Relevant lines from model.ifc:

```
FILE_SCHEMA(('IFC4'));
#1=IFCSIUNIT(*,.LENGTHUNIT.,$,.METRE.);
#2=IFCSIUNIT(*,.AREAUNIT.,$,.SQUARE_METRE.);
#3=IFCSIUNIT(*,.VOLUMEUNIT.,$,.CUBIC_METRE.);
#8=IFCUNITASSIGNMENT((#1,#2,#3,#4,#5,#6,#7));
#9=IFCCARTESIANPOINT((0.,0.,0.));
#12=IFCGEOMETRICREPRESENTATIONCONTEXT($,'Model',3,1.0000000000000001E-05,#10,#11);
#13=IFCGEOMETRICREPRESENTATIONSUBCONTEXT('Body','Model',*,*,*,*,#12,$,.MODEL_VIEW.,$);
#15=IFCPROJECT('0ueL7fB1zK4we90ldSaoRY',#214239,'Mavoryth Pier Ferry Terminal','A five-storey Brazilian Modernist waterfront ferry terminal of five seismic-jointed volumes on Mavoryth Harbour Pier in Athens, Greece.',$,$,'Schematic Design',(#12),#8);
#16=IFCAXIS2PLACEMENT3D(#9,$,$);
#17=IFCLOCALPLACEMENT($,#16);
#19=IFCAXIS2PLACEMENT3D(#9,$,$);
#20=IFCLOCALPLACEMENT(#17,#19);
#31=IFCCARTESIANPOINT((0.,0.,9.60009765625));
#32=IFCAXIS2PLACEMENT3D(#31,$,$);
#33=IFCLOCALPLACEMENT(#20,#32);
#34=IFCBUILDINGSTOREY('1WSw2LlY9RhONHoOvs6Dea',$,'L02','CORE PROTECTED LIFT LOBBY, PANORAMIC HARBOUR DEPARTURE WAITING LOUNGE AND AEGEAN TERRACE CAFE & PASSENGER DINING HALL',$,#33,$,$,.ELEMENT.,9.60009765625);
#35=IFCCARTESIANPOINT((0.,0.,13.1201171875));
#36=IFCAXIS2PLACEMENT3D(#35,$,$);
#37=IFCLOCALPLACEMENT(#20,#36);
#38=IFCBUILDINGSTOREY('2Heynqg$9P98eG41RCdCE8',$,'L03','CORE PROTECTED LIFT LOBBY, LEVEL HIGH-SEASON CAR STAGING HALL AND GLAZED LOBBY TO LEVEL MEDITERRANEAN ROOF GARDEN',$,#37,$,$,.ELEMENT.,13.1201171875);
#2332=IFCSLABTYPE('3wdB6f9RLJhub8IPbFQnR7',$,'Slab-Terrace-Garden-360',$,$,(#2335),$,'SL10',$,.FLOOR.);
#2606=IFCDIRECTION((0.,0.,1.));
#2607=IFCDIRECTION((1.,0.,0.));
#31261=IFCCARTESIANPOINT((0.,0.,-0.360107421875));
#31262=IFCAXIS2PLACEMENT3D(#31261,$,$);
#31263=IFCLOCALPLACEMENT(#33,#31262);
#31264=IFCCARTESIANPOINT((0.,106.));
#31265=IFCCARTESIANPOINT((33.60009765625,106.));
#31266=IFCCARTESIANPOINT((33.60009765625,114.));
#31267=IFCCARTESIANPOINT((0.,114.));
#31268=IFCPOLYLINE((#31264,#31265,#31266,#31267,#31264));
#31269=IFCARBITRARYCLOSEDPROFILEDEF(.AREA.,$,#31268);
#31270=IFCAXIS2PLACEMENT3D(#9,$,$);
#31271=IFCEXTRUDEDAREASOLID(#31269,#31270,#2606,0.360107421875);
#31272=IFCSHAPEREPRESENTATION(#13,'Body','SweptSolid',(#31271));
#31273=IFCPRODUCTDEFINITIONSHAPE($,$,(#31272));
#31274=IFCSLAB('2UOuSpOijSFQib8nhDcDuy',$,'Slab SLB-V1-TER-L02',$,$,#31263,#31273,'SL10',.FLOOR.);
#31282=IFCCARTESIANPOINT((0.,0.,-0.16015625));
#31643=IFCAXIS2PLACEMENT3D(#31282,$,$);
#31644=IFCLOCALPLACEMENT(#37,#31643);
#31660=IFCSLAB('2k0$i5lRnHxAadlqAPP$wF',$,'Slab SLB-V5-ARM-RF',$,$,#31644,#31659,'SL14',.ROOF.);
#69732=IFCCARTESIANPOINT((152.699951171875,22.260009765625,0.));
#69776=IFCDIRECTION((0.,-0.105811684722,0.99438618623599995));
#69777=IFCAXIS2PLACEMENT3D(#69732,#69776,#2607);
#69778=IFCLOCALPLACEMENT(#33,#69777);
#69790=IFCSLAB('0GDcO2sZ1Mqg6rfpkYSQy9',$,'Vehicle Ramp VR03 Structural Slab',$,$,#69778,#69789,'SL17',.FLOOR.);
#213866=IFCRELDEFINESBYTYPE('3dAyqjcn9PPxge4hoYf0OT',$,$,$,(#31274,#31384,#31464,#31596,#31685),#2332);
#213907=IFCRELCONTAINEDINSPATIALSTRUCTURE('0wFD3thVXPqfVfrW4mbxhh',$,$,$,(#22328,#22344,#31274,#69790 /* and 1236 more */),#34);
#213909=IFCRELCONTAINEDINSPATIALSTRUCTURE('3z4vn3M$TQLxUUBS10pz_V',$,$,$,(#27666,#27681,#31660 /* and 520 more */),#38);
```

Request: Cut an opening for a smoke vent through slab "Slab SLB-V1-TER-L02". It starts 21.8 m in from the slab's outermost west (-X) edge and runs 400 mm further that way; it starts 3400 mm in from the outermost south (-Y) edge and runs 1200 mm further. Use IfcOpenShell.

```python
import numpy as np
import ifcopenshell
import ifcopenshell.api.feature
import ifcopenshell.api.geometry
import ifcopenshell.api.root
import ifcopenshell.geom
import ifcopenshell.util.placement
import ifcopenshell.util.representation
import ifcopenshell.util.shape
import ifcopenshell.util.unit

model = ifcopenshell.open("model.ifc")
unit_scale = ifcopenshell.util.unit.calculate_unit_scale(model)
settings = ifcopenshell.geom.settings()


def volume(element):
    """Net volume in cubic metres, openings subtracted."""
    shape = ifcopenshell.geom.create_shape(settings, element)
    return ifcopenshell.util.shape.get_volume(shape.geometry)


slab = model.by_guid("2UOuSpOijSFQib8nhDcDuy")
before = volume(slab)

# Extent in the slab's own axes, in metres. The edges named are its -X and -Y sides.
slab_shape = ifcopenshell.geom.create_shape(settings, slab)
vertices = ifcopenshell.util.shape.get_vertices(slab_shape.geometry)
x_min, y_min, bottom = vertices.min(axis=0)
top = vertices[:, 2].max()

opening = ifcopenshell.api.root.create_entity(model, ifc_class="IfcOpeningElement", name="Smoke vent opening", predefined_type="OPENING")
context = ifcopenshell.util.representation.get_context(model, "Model", "Body", "MODEL_VIEW")
width, depth = 0.4, 1.2
outline = [(0.0, 0.0), (width, 0.0), (width, depth), (0.0, depth), (0.0, 0.0)]
# Overshoot both faces by 50 mm so the cut is clean.
shape = ifcopenshell.api.geometry.add_slab_representation(
    model, context=context, depth=top - bottom + 0.1, polyline=outline
)
ifcopenshell.api.geometry.assign_representation(model, product=opening, representation=shape)

matrix = ifcopenshell.util.placement.get_local_placement(slab.ObjectPlacement)
matrix[:, 3] = matrix @ np.append(np.array([x_min + 21.8, y_min + 3.4, bottom - 0.05]) / unit_scale, 1.0)
ifcopenshell.api.geometry.edit_object_placement(model, product=opening, matrix=matrix, is_si=False)
ifcopenshell.api.feature.add_feature(model, feature=opening, element=slab)

after = volume(slab)

print(f"slab volume {before:.3f} -> {after:.3f} m3")

model.write("model-out.ifc")
```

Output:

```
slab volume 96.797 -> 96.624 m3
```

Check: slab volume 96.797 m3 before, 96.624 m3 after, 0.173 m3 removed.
